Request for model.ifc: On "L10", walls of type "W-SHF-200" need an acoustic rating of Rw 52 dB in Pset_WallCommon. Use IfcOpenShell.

First a look at what the model holds.

```python
import ifcopenshell
import ifcopenshell.util.element

model = ifcopenshell.open("model.ifc")
print(model.schema)
storey = next(s for s in model.by_type("IfcBuildingStorey") if s.Name == "L10")
walls = [e for e in ifcopenshell.util.element.get_decomposition(storey) if e.is_a("IfcWall")]
seen = {}
for e in walls:
    element_type = ifcopenshell.util.element.get_type(e)
    key = (element_type.Name if element_type != e and element_type else None, ifcopenshell.util.element.get_pset(e, "Pset_WallCommon", "AcousticRating"))
    seen[key] = seen.get(key, 0) + 1
for (name, value), count in sorted(seen.items(), key=str):
    print(count, "x", name, "|", value)
```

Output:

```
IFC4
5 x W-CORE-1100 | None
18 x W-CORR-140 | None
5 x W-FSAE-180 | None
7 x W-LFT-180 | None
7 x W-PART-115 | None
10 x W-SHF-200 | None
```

```python
import ifcopenshell
import ifcopenshell.api.pset
import ifcopenshell.util.element

model = ifcopenshell.open("model.ifc")

storey = next(s for s in model.by_type("IfcBuildingStorey") if s.Name == "L10")
walls = [e for e in ifcopenshell.util.element.get_decomposition(storey) if e.is_a("IfcWall")]

count = 0
for e in walls:
    element_type = ifcopenshell.util.element.get_type(e)
    if element_type in (None, e) or element_type.Name != "W-SHF-200":
        continue
    found = ifcopenshell.util.element.get_pset(e, "Pset_WallCommon", should_inherit=False)
    if found:
        pset = model.by_id(found["id"])
        if len(ifcopenshell.util.element.get_elements_by_pset(pset)) > 1:
            pset = ifcopenshell.api.pset.unshare_pset(model, products=[e], pset=pset)[0]
    else:
        pset = ifcopenshell.api.pset.add_pset(model, product=e, name="Pset_WallCommon")
    ifcopenshell.api.pset.edit_pset(model, pset=pset, properties={"AcousticRating": "Rw 52 dB"})
    count += 1

print(count, "walls updated")

model.write("model_updated.ifc")
```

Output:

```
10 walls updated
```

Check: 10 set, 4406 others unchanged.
